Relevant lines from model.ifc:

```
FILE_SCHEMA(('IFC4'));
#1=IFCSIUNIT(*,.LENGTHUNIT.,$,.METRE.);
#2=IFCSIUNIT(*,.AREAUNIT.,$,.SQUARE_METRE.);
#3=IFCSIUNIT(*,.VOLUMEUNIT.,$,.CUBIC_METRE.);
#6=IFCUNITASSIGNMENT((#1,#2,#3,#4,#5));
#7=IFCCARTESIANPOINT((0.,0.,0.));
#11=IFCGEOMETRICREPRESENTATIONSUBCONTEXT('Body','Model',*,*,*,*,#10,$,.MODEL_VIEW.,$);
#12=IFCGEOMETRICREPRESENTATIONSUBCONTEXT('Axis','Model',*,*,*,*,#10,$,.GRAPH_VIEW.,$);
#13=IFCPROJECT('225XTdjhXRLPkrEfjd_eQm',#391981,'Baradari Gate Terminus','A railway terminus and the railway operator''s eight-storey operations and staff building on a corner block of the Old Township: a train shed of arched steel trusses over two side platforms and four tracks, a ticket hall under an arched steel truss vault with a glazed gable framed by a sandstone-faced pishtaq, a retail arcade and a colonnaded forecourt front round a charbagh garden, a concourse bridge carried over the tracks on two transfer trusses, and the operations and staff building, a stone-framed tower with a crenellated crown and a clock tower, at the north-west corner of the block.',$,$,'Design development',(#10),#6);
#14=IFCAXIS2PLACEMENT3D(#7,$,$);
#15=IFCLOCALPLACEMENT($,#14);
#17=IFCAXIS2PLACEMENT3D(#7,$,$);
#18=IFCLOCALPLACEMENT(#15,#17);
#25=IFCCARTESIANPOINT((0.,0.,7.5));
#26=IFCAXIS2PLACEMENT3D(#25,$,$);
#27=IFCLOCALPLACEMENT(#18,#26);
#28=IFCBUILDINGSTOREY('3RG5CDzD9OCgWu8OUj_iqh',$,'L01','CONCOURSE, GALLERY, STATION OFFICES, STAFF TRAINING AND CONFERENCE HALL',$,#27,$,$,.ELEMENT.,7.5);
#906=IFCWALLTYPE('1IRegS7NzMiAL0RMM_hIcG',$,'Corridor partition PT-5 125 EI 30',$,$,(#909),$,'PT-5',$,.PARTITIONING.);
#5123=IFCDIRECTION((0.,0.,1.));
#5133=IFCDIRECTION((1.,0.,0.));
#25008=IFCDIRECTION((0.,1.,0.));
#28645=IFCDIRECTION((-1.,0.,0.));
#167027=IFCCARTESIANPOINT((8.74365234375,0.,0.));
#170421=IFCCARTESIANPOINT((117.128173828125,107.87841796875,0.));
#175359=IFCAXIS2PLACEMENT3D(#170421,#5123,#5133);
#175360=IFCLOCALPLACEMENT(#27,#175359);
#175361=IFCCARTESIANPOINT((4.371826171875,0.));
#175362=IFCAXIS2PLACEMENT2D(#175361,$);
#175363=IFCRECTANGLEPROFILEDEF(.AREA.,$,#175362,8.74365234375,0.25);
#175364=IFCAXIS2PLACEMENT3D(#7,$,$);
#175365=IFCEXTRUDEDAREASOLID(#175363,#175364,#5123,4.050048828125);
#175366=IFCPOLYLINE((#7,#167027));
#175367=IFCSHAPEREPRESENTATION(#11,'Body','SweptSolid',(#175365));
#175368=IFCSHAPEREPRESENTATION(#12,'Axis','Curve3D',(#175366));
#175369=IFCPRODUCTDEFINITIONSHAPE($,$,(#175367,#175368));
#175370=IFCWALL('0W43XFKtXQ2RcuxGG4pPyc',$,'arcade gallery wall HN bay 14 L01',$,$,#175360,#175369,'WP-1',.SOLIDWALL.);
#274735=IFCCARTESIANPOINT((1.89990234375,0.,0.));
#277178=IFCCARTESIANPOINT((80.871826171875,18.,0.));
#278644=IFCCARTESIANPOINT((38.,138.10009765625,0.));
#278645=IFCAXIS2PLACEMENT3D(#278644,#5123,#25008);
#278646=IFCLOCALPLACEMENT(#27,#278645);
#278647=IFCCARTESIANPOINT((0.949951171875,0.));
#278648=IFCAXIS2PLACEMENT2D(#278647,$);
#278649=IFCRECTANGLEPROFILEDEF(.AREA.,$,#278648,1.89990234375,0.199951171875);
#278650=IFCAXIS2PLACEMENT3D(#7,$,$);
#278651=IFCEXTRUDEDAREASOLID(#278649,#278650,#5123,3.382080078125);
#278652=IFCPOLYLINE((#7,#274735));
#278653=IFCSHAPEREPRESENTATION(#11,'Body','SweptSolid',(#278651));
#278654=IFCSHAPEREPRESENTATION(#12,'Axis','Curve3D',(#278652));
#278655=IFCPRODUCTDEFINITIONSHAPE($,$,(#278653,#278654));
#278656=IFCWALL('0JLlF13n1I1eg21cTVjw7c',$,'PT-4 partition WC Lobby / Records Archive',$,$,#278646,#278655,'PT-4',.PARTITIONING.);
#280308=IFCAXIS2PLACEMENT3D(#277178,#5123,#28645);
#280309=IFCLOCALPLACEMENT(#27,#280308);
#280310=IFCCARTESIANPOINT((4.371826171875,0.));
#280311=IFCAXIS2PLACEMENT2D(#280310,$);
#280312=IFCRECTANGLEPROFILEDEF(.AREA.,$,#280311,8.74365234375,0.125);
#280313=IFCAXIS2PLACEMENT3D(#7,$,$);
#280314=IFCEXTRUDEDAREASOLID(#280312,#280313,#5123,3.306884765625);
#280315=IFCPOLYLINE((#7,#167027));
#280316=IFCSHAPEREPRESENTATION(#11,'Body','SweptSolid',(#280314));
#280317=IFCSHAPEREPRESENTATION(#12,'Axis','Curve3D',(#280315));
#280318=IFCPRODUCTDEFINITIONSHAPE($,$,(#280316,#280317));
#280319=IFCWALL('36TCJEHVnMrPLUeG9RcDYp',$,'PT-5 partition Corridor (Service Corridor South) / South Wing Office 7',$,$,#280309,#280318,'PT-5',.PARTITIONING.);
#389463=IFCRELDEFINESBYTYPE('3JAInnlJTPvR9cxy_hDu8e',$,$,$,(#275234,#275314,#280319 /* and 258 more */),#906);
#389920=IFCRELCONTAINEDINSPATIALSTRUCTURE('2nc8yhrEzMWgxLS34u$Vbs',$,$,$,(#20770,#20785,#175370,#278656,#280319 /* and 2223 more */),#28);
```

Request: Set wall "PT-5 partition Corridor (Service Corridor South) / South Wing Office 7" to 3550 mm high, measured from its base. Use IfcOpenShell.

```python
import ifcopenshell
import ifcopenshell.geom
import ifcopenshell.util.representation
import ifcopenshell.util.shape

model = ifcopenshell.open("model.ifc")
settings = ifcopenshell.geom.settings()


def volume(element):
    """Net volume in cubic metres, openings subtracted."""
    shape = ifcopenshell.geom.create_shape(settings, element)
    return ifcopenshell.util.shape.get_volume(shape.geometry)


wall = model.by_guid("36TCJEHVnMrPLUeG9RcDYp")
before = volume(wall)

body = ifcopenshell.util.representation.get_representation(wall, "Model", "Body")
solid = body.Items[0]
old_height = solid.Depth
solid.Depth = 3.55
after = volume(wall)

print(f"height {old_height:g} -> {solid.Depth:g}, volume {before:.3f} -> {after:.3f} m3")

model.write("model_updated.ifc")
```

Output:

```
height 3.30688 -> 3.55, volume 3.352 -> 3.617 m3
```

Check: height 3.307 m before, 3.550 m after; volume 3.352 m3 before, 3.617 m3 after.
